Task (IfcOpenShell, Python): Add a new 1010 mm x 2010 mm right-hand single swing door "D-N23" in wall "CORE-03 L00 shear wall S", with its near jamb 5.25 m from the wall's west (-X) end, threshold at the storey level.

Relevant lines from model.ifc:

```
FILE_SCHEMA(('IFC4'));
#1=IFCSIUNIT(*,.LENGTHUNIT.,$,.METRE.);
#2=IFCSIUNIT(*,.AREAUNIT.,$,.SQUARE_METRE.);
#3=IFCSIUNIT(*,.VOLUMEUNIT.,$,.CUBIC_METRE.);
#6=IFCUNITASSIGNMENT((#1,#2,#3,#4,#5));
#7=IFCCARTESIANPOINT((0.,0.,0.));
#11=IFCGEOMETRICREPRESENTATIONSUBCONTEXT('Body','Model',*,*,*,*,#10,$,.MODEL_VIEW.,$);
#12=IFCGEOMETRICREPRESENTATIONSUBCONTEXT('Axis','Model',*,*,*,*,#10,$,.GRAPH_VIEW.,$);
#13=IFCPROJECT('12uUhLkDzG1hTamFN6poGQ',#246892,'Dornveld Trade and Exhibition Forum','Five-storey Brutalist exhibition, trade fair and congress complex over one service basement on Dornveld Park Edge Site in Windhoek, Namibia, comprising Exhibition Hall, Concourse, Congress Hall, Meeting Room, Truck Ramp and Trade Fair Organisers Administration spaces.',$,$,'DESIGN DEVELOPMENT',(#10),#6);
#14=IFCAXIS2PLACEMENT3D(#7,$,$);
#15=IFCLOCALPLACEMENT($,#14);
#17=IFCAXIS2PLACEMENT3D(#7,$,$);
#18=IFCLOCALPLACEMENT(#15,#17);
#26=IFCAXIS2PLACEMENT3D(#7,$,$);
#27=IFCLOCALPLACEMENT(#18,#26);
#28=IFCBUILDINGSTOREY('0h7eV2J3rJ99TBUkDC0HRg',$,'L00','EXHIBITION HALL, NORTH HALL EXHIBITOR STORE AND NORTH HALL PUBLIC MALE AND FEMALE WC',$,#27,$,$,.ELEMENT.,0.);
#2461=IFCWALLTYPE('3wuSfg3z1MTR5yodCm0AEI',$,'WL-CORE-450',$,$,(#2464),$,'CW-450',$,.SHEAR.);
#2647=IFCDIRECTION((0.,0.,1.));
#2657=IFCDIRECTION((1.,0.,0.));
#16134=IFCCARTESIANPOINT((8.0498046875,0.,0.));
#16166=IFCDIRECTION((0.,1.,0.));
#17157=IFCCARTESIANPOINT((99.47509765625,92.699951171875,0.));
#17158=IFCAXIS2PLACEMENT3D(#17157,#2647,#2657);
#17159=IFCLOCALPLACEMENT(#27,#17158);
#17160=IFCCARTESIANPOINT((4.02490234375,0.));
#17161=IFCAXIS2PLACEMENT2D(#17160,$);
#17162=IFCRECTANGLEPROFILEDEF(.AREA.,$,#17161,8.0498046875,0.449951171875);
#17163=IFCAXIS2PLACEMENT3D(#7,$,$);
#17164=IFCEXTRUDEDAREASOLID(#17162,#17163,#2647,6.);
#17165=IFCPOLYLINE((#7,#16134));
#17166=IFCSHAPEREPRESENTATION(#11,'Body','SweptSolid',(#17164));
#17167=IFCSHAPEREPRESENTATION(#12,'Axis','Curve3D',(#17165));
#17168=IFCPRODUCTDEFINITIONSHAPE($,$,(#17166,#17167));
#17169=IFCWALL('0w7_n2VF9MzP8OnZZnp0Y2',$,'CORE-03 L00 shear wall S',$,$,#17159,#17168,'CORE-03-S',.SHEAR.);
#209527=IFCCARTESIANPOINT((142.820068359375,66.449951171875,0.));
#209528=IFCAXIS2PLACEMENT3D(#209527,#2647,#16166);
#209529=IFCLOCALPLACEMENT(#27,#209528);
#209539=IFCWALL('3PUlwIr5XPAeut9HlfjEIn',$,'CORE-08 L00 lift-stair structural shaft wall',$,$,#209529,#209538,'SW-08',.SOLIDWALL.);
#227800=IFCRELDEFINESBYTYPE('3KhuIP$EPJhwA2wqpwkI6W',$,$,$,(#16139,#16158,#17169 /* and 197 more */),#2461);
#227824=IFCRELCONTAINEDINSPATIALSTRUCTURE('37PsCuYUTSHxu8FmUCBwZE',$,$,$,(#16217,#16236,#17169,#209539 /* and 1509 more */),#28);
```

```python
import numpy as np
import ifcopenshell
import ifcopenshell.api.feature
import ifcopenshell.api.geometry
import ifcopenshell.api.root
import ifcopenshell.api.spatial
import ifcopenshell.geom
import ifcopenshell.util.element
import ifcopenshell.util.placement
import ifcopenshell.util.representation
import ifcopenshell.util.shape
import ifcopenshell.util.unit

model = ifcopenshell.open("model.ifc")
unit_scale = ifcopenshell.util.unit.calculate_unit_scale(model)
settings = ifcopenshell.geom.settings()


def volume(element):
    """Net volume in cubic metres, openings subtracted."""
    shape = ifcopenshell.geom.create_shape(settings, element)
    return ifcopenshell.util.shape.get_volume(shape.geometry)


wall = model.by_id(17169)
storey = ifcopenshell.util.element.get_container(wall, ifc_class="IfcBuildingStorey")
context = ifcopenshell.util.representation.get_context(model, "Model", "Body", "MODEL_VIEW")
before = volume(wall)

width, height, from_end, sill = 1.01, 2.01, 5.25, 0.0  # metres

# The wall runs along its own X axis, and the end named is its -X end.
wall_shape = ifcopenshell.geom.create_shape(settings, wall)
x, y, z = ifcopenshell.util.shape.get_vertices(wall_shape.geometry).T
start = x.min() + from_end
face, thickness = float(y.min()), float(y.max() - y.min())
wall_matrix = ifcopenshell.util.placement.get_local_placement(wall.ObjectPlacement)
level = ifcopenshell.util.placement.get_local_placement(storey.ObjectPlacement)[2, 3]


def in_wall(x, y):
    """Placement at x, y metres in the wall's axes, at sill height."""
    matrix = wall_matrix.copy()
    matrix[:, 3] = wall_matrix @ np.array([x / unit_scale, y / unit_scale, 0.0, 1.0])
    matrix[2, 3] = level + sill / unit_scale
    return matrix


# Opening: a box that overshoots both wall faces by 50 mm.
opening = ifcopenshell.api.root.create_entity(model, ifc_class="IfcOpeningElement", predefined_type="OPENING")
box = ifcopenshell.api.geometry.add_wall_representation(
    model, context=context, length=width, height=height, thickness=thickness + 0.1
)
ifcopenshell.api.geometry.assign_representation(model, product=opening, representation=box)
ifcopenshell.api.geometry.edit_object_placement(model, product=opening, matrix=in_wall(start, face - 0.05), is_si=False)
ifcopenshell.api.feature.add_feature(model, feature=opening, element=wall)

door = ifcopenshell.api.root.create_entity(model, ifc_class="IfcDoor", name="D-N23", predefined_type="DOOR")
door.OverallWidth, door.OverallHeight = width / unit_scale, height / unit_scale
door.OperationType = "SINGLE_SWING_RIGHT"
body = ifcopenshell.api.geometry.add_door_representation(
    model,
    context=context,
    overall_width=door.OverallWidth,
    overall_height=door.OverallHeight,
    operation_type="SINGLE_SWING_RIGHT",
    lining_properties={"LiningDepth": thickness / unit_scale, "ThresholdDepth": thickness / unit_scale},
)
ifcopenshell.api.geometry.assign_representation(model, product=door, representation=body)
ifcopenshell.api.spatial.assign_container(model, products=[door], relating_structure=storey)
ifcopenshell.api.feature.add_filling(model, opening=opening, element=door)

# The lining spans the wall, so the door starts at the wall face.
ifcopenshell.api.geometry.edit_object_placement(model, product=door, matrix=in_wall(start, face), is_si=False)

after = volume(wall)

print(f"wall volume {before:.3f} -> {after:.3f} m3")

model.write("model-out.ifc")
```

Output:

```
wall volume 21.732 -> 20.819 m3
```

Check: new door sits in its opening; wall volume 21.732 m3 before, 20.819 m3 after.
